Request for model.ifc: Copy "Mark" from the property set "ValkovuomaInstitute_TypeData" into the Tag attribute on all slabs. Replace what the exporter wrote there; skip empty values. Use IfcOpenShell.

First a look at what the model holds.

```python
import ifcopenshell
import ifcopenshell.util.element

model = ifcopenshell.open("model.ifc")
print(model.schema)
slabs = model.by_type("IfcSlab")
print(len(slabs), "slabs")
for e in slabs[:8]:
    source = ifcopenshell.util.element.get_pset(e, "ValkovuomaInstitute_TypeData", "Mark")
    target = e.Tag
    print(e.id(), repr(source), repr(target), sep=" | ")
```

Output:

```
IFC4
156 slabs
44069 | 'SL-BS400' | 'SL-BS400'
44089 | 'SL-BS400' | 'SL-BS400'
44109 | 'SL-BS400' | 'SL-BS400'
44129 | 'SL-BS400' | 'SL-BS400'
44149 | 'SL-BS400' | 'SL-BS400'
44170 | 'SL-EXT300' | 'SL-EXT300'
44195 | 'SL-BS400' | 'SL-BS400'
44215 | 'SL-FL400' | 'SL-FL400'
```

```python
import ifcopenshell
import ifcopenshell.util.element

model = ifcopenshell.open("model.ifc")

count = 0
for e in model.by_type("IfcSlab"):
    value = ifcopenshell.util.element.get_pset(e, "ValkovuomaInstitute_TypeData", "Mark")
    current = e.Tag
    if not value or not value.strip() or current == value:
        continue
    e.Tag = value
    count += 1

print(count, "slabs updated")

model.write("model_updated.ifc")
```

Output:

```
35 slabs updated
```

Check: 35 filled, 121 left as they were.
